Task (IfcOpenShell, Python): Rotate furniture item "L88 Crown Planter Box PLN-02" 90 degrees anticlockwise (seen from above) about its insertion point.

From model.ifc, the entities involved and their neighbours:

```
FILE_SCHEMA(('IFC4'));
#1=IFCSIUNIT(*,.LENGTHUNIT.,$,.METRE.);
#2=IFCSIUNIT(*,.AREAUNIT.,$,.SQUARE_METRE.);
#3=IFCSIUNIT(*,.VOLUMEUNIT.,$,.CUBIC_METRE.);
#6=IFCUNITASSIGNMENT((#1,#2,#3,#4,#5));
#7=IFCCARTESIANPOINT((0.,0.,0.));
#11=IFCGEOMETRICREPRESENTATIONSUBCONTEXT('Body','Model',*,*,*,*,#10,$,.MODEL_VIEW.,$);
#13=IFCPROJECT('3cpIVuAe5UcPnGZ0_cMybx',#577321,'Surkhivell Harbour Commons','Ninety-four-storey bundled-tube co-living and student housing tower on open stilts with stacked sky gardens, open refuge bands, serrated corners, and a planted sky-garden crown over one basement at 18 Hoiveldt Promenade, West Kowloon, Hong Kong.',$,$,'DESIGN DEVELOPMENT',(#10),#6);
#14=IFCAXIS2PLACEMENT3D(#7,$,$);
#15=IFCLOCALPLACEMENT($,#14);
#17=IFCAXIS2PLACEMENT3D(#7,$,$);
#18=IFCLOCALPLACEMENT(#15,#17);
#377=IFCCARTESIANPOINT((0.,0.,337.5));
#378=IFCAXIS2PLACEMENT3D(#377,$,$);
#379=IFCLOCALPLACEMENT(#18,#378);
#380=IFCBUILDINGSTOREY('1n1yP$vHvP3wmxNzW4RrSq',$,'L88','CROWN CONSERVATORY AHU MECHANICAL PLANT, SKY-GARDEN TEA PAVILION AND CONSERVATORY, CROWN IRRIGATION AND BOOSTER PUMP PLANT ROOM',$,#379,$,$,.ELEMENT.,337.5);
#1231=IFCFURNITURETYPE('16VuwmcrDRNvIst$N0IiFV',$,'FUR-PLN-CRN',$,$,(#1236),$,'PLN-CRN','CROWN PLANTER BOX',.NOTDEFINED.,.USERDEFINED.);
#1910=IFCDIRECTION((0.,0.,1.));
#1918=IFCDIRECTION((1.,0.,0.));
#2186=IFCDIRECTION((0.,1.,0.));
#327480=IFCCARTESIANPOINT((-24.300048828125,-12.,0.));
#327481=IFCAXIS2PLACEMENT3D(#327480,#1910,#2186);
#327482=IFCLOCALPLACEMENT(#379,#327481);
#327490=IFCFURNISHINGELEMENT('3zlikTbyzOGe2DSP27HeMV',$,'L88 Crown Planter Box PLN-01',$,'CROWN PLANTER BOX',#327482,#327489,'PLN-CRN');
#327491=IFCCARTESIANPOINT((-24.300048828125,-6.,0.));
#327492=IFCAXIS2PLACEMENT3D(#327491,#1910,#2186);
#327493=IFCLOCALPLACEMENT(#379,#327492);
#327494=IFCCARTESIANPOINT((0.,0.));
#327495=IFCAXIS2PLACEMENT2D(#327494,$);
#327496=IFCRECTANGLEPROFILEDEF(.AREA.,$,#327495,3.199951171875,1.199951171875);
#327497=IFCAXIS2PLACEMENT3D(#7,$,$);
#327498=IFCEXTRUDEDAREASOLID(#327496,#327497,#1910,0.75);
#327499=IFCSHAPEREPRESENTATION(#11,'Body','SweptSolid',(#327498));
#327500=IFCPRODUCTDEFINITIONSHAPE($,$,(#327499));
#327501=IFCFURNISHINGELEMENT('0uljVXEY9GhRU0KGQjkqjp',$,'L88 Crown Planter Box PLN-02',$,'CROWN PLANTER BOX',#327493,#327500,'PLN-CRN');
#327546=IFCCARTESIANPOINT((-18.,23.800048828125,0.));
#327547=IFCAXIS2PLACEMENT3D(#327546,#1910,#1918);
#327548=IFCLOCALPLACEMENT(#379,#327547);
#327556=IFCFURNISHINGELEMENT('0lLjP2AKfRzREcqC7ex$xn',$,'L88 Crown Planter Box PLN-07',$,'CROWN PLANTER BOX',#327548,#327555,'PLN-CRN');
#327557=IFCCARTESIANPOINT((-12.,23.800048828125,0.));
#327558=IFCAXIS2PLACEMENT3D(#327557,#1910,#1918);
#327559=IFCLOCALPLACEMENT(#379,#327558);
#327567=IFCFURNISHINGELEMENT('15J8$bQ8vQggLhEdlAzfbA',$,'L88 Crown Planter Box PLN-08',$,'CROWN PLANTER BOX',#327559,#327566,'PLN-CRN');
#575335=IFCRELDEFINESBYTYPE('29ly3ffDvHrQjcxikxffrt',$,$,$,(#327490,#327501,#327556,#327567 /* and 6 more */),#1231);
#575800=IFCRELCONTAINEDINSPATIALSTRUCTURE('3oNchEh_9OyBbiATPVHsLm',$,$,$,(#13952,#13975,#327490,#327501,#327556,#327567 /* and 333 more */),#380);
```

```python
import ifcopenshell
import ifcopenshell.api.geometry
import ifcopenshell.util.placement

model = ifcopenshell.open("model.ifc")

item = model.by_guid("0uljVXEY9GhRU0KGQjkqjp")
matrix = ifcopenshell.util.placement.get_local_placement(item.ObjectPlacement)
matrix = matrix @ ifcopenshell.util.placement.rotation(90, "Z")
ifcopenshell.api.geometry.edit_object_placement(model, product=item, matrix=matrix, is_si=False)

print(ifcopenshell.util.placement.get_local_placement(item.ObjectPlacement).round(3) + 0.0)

model.write("model_v2.ifc")
```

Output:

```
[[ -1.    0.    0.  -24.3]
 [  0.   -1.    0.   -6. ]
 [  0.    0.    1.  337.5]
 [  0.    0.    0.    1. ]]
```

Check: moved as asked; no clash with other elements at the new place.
